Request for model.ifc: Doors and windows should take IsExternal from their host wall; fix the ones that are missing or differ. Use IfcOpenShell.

First a look at what the model holds.

```python
import ifcopenshell
import ifcopenshell.util.element

model = ifcopenshell.open("model.ifc")
print(model.schema)
seen = {}
for e in model.by_type("IfcDoor") + model.by_type("IfcWindow"):
    if not e.FillsVoids:
        continue
    host = e.FillsVoids[0].RelatingOpeningElement.VoidsElements[0].RelatingBuildingElement
    own = ifcopenshell.util.element.get_pset(e, f"Pset_{e.is_a()[3:].removesuffix('StandardCase')}Common", "IsExternal")
    wall = ifcopenshell.util.element.get_pset(host, "Pset_WallCommon", "IsExternal")
    seen[e.is_a(), own, wall] = seen.get((e.is_a(), own, wall), 0) + 1
for (cls, own, wall), count in sorted(seen.items(), key=str):
    print(count, cls, "IsExternal:", own, "| host wall:", wall)
```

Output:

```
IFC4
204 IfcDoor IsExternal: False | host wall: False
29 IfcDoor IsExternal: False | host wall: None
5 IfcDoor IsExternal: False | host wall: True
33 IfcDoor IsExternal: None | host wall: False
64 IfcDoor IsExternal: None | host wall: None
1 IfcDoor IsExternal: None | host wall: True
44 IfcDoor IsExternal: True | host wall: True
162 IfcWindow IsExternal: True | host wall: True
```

```python
import ifcopenshell
import ifcopenshell.api.pset
import ifcopenshell.util.element

model = ifcopenshell.open("model.ifc")

count = 0
for ifc_class, pset_name in (("IfcDoor", "Pset_DoorCommon"), ("IfcWindow", "Pset_WindowCommon")):
    for e in model.by_type(ifc_class):
        if not e.FillsVoids:
            continue
        host = e.FillsVoids[0].RelatingOpeningElement.VoidsElements[0].RelatingBuildingElement
        external = ifcopenshell.util.element.get_pset(host, "Pset_WallCommon", "IsExternal")
        if external is None or ifcopenshell.util.element.get_pset(e, pset_name, "IsExternal") == external:
            continue
        pset = ifcopenshell.api.pset.add_pset(model, product=e, name=pset_name)
        ifcopenshell.api.pset.edit_pset(model, pset=pset, properties={"IsExternal": external})
        count += 1

print(count, "updated")

model.write("model_rev.ifc")
```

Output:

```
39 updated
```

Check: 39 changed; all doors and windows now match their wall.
